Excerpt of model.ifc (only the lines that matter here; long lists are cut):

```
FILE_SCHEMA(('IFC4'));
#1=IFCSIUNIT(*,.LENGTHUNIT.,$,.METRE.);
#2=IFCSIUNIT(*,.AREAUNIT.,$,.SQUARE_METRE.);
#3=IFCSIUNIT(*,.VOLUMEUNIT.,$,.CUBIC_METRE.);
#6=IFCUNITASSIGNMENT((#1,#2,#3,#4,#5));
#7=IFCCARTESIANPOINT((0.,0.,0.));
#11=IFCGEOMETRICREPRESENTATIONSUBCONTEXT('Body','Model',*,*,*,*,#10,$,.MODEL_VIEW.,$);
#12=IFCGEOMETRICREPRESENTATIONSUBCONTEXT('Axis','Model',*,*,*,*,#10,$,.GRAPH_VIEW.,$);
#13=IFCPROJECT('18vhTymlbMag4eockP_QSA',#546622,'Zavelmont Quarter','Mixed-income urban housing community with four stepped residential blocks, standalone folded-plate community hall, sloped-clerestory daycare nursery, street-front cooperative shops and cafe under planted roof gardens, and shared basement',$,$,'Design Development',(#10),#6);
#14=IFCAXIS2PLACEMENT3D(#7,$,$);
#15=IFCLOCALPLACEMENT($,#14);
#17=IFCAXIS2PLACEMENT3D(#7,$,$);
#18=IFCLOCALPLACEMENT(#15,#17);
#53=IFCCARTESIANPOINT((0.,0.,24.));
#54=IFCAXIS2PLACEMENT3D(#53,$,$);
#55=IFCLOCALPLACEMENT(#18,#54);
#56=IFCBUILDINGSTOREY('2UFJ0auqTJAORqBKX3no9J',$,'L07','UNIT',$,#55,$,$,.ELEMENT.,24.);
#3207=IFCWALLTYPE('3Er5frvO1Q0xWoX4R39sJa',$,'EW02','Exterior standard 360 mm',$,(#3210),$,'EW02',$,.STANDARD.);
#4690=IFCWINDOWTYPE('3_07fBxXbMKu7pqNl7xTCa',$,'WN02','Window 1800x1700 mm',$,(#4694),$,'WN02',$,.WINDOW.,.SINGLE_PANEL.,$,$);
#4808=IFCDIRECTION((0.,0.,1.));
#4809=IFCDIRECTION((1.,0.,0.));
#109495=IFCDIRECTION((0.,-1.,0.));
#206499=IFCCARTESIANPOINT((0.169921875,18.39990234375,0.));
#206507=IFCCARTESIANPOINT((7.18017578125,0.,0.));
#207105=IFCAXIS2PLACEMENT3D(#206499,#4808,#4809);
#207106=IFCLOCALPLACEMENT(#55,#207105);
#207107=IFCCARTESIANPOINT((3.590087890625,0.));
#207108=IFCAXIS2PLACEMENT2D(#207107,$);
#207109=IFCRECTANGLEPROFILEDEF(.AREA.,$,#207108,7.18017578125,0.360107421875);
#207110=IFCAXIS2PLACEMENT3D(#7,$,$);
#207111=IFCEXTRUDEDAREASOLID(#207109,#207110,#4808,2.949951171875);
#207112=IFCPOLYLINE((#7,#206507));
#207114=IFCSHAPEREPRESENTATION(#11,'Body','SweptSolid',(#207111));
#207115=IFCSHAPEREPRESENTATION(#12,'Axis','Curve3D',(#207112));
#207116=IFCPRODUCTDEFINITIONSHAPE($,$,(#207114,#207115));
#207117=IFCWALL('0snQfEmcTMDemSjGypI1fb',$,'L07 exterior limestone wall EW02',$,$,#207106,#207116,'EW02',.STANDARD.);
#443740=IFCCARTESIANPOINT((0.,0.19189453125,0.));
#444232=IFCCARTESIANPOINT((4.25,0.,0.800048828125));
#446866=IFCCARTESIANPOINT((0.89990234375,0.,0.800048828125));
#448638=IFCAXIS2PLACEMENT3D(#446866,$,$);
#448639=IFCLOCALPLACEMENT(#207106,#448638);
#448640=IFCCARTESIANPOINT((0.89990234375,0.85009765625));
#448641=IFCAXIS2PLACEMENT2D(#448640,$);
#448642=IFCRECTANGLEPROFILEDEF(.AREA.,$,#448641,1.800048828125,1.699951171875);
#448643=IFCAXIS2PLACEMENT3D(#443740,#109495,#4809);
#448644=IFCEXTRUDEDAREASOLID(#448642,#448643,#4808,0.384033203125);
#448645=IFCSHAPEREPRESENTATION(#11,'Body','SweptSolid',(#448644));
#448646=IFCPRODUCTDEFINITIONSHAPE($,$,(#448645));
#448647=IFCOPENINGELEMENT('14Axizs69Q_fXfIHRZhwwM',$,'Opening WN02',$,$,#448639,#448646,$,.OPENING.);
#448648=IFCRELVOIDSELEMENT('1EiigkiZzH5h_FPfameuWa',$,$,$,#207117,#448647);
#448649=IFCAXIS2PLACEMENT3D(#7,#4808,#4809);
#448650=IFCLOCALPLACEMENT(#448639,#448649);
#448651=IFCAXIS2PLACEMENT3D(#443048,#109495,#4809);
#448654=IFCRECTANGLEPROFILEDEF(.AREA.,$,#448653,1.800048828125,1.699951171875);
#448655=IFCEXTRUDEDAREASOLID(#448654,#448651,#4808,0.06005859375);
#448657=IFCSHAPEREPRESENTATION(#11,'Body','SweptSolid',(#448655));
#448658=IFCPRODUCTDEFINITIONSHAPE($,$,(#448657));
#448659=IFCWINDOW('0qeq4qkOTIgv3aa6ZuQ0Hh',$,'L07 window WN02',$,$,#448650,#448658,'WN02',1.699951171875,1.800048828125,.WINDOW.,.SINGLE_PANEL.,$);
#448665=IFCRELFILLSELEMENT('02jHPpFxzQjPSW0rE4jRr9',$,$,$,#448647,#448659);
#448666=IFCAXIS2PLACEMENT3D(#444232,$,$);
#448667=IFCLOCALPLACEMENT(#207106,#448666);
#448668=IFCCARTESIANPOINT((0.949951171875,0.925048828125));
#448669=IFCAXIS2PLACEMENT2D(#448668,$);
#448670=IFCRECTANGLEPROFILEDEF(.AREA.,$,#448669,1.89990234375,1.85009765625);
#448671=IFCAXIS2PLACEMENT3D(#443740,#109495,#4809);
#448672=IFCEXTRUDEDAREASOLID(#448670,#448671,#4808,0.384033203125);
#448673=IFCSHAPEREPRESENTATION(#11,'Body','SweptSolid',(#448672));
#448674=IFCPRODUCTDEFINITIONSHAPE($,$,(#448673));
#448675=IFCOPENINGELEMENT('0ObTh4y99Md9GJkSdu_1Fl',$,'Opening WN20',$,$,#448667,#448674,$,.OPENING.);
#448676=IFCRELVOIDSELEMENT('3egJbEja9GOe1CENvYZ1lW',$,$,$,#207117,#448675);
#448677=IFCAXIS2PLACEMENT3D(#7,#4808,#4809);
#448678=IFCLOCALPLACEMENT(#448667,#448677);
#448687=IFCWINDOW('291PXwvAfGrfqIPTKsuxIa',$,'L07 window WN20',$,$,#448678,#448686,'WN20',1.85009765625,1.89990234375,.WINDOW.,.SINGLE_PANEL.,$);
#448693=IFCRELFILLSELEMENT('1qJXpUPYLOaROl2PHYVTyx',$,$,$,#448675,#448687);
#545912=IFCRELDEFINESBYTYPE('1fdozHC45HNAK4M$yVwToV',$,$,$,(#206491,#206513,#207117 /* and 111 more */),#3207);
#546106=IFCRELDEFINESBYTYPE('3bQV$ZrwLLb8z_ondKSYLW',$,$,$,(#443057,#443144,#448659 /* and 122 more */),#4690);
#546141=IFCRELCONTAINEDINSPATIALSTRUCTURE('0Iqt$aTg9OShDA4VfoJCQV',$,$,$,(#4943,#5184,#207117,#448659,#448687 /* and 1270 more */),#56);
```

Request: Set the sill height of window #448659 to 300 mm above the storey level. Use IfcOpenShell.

```python
import numpy as np
import ifcopenshell
import ifcopenshell.api.geometry
import ifcopenshell.geom
import ifcopenshell.util.element
import ifcopenshell.util.placement
import ifcopenshell.util.shape
import ifcopenshell.util.unit

model = ifcopenshell.open("model.ifc")
unit_scale = ifcopenshell.util.unit.calculate_unit_scale(model)

window = model.by_id(448659)
opening = window.FillsVoids[0].RelatingOpeningElement
storey = ifcopenshell.util.element.get_container(window, ifc_class="IfcBuildingStorey")
level = ifcopenshell.util.placement.get_local_placement(storey.ObjectPlacement)[2, 3]

# The opening's origin need not be at the sill, so measure its lowest point.
shape = ifcopenshell.geom.create_shape(ifcopenshell.geom.settings(), opening)
bottom = ifcopenshell.util.shape.get_shape_bottom_elevation(shape, shape.geometry) / unit_scale
dz = level + 0.3 / unit_scale - bottom

shift = np.array([0.0, 0.0, dz])
# The window is placed relative to its opening, so it follows when the opening moves.
matrix = ifcopenshell.util.placement.get_local_placement(opening.ObjectPlacement)
matrix[:3, 3] += shift
ifcopenshell.api.geometry.edit_object_placement(
    model, product=opening, matrix=matrix, is_si=False, should_transform_children=True
)

print(f"moved by {dz * unit_scale:+.3f} m")

model.write("model_edited.ifc")
```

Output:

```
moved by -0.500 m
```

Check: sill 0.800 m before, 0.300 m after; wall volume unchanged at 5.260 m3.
